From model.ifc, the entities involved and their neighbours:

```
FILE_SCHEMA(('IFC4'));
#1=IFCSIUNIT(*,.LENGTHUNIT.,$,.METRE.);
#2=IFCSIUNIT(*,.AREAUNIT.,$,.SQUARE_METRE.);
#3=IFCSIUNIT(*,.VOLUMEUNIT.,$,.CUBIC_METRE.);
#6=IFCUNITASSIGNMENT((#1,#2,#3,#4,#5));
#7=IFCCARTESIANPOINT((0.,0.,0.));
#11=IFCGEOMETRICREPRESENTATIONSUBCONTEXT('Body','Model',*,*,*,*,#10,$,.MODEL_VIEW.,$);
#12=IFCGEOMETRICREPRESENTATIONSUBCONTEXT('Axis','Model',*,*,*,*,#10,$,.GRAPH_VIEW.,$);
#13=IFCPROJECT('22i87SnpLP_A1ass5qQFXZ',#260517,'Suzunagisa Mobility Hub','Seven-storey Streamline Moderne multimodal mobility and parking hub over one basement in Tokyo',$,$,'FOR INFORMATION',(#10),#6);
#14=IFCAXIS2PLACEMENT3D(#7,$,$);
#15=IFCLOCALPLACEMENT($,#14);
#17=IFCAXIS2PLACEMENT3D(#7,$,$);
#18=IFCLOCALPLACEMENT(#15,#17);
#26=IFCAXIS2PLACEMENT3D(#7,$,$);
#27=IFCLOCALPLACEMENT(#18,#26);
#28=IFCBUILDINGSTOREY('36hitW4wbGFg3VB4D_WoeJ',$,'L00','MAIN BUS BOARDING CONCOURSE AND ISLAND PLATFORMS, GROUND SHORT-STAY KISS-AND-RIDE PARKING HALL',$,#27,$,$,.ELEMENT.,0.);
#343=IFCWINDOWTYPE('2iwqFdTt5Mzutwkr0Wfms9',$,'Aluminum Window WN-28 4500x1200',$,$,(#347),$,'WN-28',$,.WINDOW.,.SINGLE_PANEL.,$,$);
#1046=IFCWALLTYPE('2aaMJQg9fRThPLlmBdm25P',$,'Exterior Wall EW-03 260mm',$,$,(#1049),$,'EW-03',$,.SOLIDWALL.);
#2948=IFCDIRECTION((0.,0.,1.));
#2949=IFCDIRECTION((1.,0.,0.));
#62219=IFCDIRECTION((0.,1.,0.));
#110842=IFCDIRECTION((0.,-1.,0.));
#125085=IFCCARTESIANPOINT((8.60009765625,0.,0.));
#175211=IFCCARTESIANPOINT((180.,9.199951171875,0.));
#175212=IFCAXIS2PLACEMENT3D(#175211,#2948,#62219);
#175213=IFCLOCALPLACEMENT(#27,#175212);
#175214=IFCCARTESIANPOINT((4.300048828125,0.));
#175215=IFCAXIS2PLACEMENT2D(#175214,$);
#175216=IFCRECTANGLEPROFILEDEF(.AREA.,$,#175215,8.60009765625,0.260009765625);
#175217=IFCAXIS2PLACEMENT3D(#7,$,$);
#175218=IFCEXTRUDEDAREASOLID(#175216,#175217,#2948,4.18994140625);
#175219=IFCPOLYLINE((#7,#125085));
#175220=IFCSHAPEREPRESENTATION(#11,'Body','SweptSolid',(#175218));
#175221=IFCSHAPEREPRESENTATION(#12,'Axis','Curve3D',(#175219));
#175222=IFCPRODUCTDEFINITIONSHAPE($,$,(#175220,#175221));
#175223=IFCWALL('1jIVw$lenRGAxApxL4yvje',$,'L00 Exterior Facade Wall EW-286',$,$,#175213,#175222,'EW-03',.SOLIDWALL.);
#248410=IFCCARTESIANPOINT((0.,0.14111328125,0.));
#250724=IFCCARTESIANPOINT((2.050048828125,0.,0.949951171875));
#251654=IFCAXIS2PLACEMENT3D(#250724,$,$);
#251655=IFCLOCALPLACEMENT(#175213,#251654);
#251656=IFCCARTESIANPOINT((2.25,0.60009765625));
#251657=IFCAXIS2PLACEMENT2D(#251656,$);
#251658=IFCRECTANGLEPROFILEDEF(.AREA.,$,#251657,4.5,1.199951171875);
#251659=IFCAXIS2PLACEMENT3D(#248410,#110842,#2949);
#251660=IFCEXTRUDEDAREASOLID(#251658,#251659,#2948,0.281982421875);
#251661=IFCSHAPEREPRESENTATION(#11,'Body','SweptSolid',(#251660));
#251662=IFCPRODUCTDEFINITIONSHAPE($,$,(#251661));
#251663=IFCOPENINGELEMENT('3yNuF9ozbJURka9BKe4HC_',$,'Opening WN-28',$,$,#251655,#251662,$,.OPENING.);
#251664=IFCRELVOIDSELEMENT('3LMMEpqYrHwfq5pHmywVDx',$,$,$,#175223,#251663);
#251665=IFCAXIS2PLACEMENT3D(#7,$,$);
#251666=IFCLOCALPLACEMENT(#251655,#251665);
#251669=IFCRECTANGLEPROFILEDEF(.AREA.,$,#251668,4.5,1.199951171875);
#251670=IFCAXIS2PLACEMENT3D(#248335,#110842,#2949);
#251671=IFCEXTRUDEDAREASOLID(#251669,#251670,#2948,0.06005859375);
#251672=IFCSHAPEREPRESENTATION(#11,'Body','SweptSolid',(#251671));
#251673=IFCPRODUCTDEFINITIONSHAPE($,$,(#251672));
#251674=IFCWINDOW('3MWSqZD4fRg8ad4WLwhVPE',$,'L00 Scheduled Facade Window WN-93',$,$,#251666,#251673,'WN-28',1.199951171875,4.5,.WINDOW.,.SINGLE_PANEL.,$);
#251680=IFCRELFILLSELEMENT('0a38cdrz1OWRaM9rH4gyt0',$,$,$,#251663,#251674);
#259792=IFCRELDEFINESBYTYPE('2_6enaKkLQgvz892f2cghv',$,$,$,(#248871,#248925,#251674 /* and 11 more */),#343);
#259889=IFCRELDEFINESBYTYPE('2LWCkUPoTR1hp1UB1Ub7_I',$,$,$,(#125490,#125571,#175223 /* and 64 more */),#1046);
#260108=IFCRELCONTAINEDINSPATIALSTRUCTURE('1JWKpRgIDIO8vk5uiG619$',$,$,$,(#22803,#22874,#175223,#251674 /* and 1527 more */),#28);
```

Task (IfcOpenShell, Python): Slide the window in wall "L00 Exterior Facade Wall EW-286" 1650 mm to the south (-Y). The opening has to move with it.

```python
import ifcopenshell
import ifcopenshell.api.geometry
import ifcopenshell.util.placement
import ifcopenshell.util.unit

model = ifcopenshell.open("model.ifc")
unit_scale = ifcopenshell.util.unit.calculate_unit_scale(model)

window = model.by_guid("3MWSqZD4fRg8ad4WLwhVPE")
opening = window.FillsVoids[0].RelatingOpeningElement
wall = opening.VoidsElements[0].RelatingBuildingElement

wall_matrix = ifcopenshell.util.placement.get_local_placement(wall.ObjectPlacement)
shift = wall_matrix[:3, 0] * -1.65 / unit_scale
before = ifcopenshell.util.placement.get_local_placement(window.ObjectPlacement)[:3, 3].copy()

# The window is placed relative to its opening, so it follows when the opening moves.
matrix = ifcopenshell.util.placement.get_local_placement(opening.ObjectPlacement)
matrix[:3, 3] += shift
ifcopenshell.api.geometry.edit_object_placement(
    model, product=opening, matrix=matrix, is_si=False, should_transform_children=True
)

after = ifcopenshell.util.placement.get_local_placement(window.ObjectPlacement)[:3, 3]
print("window moved by", (after - before).round(3) + 0.0)

model.write("model_rev.ifc")
```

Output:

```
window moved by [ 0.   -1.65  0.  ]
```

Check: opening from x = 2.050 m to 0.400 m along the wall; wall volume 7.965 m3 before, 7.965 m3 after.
